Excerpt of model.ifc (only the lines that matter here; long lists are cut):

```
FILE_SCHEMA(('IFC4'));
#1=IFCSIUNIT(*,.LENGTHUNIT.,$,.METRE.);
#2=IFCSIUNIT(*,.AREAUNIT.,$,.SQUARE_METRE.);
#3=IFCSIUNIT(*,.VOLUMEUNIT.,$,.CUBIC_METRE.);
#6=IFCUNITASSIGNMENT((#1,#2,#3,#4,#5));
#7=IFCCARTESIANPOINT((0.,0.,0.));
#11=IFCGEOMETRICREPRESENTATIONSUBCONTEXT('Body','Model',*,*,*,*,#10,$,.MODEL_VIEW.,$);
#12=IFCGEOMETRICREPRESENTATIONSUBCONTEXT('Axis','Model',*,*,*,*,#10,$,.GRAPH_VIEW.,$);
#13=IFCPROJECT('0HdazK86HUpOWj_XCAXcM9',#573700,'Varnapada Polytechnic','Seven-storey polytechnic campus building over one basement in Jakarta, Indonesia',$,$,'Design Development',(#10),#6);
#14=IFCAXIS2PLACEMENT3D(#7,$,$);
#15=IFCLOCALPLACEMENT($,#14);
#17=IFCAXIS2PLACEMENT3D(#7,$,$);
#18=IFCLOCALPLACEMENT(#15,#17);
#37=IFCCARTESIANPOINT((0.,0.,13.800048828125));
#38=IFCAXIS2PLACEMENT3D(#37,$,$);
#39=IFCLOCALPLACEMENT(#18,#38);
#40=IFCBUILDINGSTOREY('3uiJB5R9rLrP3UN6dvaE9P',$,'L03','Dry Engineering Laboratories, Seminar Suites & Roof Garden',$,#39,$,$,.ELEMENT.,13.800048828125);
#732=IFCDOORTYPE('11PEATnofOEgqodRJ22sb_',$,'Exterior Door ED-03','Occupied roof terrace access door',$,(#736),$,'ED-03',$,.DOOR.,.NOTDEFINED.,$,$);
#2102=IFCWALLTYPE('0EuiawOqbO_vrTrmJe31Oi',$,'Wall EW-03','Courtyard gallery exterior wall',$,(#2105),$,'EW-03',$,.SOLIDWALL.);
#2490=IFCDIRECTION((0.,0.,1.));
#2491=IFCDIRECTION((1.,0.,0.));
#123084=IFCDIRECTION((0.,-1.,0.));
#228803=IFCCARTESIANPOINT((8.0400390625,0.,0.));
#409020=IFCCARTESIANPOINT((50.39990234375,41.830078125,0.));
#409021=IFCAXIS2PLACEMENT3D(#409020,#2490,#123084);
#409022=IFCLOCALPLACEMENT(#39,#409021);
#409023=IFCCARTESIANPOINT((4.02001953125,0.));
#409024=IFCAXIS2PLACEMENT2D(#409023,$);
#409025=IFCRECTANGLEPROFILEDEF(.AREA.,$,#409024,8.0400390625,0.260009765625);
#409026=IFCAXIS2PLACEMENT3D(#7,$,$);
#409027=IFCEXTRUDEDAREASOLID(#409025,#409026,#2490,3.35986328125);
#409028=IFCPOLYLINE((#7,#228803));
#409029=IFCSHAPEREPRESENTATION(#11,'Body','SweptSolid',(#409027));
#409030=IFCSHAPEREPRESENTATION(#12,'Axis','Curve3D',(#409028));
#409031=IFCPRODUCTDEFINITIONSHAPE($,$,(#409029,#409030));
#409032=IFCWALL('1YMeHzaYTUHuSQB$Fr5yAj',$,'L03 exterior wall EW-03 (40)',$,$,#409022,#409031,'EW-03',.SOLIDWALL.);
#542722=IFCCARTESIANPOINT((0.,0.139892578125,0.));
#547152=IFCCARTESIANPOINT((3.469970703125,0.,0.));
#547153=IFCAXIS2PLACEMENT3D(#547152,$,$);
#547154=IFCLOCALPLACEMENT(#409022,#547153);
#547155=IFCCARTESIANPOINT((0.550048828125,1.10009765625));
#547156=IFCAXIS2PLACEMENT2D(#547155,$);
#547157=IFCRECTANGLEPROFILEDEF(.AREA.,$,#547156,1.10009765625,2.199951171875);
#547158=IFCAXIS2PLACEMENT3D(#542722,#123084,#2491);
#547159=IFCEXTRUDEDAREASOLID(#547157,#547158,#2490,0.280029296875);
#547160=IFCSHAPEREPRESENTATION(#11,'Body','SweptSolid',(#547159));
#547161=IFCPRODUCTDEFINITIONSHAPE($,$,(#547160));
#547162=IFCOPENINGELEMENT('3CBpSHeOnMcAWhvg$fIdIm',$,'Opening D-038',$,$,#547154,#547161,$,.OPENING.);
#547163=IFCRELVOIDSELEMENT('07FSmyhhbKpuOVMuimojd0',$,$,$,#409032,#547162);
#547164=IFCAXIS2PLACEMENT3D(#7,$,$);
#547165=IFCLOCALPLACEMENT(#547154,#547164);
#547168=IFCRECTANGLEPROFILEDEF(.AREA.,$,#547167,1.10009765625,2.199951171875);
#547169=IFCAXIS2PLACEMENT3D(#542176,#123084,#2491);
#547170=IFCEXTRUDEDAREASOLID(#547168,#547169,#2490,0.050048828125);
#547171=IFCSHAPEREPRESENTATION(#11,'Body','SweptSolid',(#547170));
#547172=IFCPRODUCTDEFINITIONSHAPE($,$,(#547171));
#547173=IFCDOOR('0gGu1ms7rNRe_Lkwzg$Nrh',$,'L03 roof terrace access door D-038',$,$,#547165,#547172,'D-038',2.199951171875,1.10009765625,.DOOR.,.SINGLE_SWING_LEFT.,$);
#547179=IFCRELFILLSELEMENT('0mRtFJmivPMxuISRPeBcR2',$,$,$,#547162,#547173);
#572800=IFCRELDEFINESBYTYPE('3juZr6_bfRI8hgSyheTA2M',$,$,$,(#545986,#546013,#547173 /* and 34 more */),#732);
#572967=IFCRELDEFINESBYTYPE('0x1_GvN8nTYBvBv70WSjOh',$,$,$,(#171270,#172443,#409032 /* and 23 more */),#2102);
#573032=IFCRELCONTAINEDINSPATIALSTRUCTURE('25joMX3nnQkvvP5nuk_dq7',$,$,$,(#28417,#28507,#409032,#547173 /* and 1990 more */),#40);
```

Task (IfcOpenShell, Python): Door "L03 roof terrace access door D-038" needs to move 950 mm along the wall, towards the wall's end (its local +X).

```python
import ifcopenshell
import ifcopenshell.api.geometry
import ifcopenshell.util.placement
import ifcopenshell.util.unit

model = ifcopenshell.open("model.ifc")
unit_scale = ifcopenshell.util.unit.calculate_unit_scale(model)

door = model.by_guid("0gGu1ms7rNRe_Lkwzg$Nrh")
opening = door.FillsVoids[0].RelatingOpeningElement
wall = opening.VoidsElements[0].RelatingBuildingElement

wall_matrix = ifcopenshell.util.placement.get_local_placement(wall.ObjectPlacement)
shift = wall_matrix[:3, 0] * 0.95 / unit_scale
before = ifcopenshell.util.placement.get_local_placement(door.ObjectPlacement)[:3, 3].copy()

# The door is placed relative to its opening, so it follows when the opening moves.
matrix = ifcopenshell.util.placement.get_local_placement(opening.ObjectPlacement)
matrix[:3, 3] += shift
ifcopenshell.api.geometry.edit_object_placement(
    model, product=opening, matrix=matrix, is_si=False, should_transform_children=True
)

after = ifcopenshell.util.placement.get_local_placement(door.ObjectPlacement)[:3, 3]
print("door moved by", (after - before).round(3) + 0.0)

model.write("model-out.ifc")
```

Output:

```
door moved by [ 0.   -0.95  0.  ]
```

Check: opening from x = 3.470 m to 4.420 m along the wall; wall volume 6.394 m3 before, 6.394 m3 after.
